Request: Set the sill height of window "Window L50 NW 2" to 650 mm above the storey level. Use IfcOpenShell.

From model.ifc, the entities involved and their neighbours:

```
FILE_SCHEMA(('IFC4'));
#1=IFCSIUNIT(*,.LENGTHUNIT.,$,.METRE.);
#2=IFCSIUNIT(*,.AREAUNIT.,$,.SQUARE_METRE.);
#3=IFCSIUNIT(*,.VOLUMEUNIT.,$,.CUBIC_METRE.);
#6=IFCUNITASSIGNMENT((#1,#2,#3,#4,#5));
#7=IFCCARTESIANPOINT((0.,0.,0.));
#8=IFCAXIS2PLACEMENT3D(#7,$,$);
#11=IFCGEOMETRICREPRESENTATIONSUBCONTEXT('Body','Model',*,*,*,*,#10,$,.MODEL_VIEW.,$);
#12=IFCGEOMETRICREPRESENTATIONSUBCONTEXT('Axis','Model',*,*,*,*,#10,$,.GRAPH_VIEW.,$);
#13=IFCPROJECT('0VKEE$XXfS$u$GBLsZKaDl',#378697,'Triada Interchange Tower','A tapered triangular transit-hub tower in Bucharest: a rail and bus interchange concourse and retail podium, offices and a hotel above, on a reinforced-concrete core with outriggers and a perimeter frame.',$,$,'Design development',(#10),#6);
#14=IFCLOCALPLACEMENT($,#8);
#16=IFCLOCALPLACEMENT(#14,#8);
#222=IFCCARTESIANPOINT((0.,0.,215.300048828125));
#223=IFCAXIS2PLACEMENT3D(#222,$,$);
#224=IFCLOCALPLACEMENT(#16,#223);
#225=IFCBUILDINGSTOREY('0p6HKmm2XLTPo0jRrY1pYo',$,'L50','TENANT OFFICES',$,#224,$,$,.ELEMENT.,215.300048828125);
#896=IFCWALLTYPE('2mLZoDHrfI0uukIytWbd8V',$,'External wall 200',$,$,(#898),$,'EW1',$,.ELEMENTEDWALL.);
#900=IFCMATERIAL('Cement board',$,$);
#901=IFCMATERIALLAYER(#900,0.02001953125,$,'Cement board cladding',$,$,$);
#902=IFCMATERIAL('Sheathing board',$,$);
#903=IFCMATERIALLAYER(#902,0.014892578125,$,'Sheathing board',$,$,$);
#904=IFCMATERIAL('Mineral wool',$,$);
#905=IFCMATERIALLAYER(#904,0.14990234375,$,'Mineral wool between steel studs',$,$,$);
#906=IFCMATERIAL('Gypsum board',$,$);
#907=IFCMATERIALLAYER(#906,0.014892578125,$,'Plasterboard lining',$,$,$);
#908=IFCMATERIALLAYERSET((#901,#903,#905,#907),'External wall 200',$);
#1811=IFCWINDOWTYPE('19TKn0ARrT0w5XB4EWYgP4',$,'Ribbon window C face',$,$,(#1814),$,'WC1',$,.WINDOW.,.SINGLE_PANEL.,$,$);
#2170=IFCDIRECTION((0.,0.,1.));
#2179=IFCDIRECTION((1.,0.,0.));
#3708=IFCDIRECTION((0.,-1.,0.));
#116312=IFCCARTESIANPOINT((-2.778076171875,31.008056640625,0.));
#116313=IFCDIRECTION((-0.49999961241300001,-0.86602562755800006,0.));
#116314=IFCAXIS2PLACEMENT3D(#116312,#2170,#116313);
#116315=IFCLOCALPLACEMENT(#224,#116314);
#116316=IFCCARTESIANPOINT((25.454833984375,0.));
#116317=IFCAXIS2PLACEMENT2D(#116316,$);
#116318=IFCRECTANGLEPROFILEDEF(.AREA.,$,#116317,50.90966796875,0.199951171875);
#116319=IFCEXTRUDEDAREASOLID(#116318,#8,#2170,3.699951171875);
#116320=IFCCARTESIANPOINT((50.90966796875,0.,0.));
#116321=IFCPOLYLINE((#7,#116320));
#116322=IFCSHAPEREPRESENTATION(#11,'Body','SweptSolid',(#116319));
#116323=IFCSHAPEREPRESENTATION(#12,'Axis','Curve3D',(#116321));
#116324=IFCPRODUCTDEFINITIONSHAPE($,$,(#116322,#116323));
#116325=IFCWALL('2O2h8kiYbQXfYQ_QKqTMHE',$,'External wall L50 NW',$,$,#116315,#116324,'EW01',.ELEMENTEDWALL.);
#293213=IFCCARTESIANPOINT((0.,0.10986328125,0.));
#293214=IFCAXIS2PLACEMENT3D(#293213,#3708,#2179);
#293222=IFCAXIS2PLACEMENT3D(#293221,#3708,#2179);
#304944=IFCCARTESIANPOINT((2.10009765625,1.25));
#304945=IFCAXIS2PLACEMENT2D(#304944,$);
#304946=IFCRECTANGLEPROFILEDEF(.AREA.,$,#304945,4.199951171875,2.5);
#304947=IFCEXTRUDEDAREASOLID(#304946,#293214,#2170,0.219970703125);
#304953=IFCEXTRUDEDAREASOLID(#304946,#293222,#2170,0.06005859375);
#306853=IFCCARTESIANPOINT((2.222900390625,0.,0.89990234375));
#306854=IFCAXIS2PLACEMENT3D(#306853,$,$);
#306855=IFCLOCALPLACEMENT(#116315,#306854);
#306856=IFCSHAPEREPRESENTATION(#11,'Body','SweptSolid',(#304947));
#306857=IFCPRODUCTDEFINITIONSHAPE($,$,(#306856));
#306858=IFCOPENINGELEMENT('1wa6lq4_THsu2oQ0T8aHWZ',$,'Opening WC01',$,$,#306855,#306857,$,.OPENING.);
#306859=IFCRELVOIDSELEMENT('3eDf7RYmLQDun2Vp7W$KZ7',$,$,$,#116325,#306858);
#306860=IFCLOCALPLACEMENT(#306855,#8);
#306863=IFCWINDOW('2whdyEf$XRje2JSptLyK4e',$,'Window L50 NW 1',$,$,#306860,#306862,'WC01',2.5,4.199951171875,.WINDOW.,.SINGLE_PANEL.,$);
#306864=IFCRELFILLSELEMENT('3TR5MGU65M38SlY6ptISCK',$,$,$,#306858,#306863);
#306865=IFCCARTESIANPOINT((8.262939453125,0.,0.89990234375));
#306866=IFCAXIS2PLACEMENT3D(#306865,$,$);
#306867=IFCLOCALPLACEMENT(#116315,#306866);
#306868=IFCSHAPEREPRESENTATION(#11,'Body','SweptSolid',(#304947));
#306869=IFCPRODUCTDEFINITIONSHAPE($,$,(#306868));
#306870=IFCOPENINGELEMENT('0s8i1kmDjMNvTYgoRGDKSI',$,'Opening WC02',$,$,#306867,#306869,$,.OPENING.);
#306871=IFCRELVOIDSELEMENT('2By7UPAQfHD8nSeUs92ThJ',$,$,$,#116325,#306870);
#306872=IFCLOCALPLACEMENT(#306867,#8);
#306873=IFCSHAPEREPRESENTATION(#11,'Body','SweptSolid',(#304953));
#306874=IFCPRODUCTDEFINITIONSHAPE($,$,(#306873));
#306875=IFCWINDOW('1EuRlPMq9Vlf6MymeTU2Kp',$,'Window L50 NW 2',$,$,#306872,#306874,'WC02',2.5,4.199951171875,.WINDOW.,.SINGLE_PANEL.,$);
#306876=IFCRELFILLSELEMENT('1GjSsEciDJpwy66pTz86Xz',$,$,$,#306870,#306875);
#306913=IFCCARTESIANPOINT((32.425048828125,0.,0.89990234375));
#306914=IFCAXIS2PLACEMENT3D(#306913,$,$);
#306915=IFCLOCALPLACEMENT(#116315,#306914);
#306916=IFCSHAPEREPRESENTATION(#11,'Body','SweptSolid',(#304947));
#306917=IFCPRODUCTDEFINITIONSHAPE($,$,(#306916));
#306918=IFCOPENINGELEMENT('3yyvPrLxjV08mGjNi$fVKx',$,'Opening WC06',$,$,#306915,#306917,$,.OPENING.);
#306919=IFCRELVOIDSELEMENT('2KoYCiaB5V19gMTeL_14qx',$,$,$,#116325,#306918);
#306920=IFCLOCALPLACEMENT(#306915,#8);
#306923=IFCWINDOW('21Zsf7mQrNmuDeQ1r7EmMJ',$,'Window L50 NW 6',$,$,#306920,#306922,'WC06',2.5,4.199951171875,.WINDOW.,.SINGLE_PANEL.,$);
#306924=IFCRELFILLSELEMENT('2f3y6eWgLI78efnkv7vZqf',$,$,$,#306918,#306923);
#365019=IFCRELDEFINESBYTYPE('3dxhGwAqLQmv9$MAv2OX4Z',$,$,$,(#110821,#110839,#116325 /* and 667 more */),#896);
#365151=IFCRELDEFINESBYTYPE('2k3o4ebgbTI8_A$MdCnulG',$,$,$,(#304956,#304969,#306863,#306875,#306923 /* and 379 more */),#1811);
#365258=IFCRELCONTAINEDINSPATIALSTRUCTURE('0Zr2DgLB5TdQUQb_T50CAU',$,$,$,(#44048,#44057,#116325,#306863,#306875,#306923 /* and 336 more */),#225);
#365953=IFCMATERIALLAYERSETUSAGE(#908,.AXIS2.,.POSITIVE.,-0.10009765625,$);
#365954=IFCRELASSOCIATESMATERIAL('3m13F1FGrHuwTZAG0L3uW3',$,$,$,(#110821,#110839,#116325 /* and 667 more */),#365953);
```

```python
import numpy as np
import ifcopenshell
import ifcopenshell.api.geometry
import ifcopenshell.geom
import ifcopenshell.util.element
import ifcopenshell.util.placement
import ifcopenshell.util.shape
import ifcopenshell.util.unit

model = ifcopenshell.open("model.ifc")
unit_scale = ifcopenshell.util.unit.calculate_unit_scale(model)

window = model.by_guid("1EuRlPMq9Vlf6MymeTU2Kp")
opening = window.FillsVoids[0].RelatingOpeningElement
storey = ifcopenshell.util.element.get_container(window, ifc_class="IfcBuildingStorey")
level = ifcopenshell.util.placement.get_local_placement(storey.ObjectPlacement)[2, 3]

# The opening's origin need not be at the sill, so measure its lowest point.
shape = ifcopenshell.geom.create_shape(ifcopenshell.geom.settings(), opening)
bottom = ifcopenshell.util.shape.get_shape_bottom_elevation(shape, shape.geometry) / unit_scale
dz = level + 0.65 / unit_scale - bottom

shift = np.array([0.0, 0.0, dz])
# The window is placed relative to its opening, so it follows when the opening moves.
matrix = ifcopenshell.util.placement.get_local_placement(opening.ObjectPlacement)
matrix[:3, 3] += shift
ifcopenshell.api.geometry.edit_object_placement(
    model, product=opening, matrix=matrix, is_si=False, should_transform_children=True
)

print(f"moved by {dz * unit_scale:+.3f} m")

model.write("model_updated.ifc")
```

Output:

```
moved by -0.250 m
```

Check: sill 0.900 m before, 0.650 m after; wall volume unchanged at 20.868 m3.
